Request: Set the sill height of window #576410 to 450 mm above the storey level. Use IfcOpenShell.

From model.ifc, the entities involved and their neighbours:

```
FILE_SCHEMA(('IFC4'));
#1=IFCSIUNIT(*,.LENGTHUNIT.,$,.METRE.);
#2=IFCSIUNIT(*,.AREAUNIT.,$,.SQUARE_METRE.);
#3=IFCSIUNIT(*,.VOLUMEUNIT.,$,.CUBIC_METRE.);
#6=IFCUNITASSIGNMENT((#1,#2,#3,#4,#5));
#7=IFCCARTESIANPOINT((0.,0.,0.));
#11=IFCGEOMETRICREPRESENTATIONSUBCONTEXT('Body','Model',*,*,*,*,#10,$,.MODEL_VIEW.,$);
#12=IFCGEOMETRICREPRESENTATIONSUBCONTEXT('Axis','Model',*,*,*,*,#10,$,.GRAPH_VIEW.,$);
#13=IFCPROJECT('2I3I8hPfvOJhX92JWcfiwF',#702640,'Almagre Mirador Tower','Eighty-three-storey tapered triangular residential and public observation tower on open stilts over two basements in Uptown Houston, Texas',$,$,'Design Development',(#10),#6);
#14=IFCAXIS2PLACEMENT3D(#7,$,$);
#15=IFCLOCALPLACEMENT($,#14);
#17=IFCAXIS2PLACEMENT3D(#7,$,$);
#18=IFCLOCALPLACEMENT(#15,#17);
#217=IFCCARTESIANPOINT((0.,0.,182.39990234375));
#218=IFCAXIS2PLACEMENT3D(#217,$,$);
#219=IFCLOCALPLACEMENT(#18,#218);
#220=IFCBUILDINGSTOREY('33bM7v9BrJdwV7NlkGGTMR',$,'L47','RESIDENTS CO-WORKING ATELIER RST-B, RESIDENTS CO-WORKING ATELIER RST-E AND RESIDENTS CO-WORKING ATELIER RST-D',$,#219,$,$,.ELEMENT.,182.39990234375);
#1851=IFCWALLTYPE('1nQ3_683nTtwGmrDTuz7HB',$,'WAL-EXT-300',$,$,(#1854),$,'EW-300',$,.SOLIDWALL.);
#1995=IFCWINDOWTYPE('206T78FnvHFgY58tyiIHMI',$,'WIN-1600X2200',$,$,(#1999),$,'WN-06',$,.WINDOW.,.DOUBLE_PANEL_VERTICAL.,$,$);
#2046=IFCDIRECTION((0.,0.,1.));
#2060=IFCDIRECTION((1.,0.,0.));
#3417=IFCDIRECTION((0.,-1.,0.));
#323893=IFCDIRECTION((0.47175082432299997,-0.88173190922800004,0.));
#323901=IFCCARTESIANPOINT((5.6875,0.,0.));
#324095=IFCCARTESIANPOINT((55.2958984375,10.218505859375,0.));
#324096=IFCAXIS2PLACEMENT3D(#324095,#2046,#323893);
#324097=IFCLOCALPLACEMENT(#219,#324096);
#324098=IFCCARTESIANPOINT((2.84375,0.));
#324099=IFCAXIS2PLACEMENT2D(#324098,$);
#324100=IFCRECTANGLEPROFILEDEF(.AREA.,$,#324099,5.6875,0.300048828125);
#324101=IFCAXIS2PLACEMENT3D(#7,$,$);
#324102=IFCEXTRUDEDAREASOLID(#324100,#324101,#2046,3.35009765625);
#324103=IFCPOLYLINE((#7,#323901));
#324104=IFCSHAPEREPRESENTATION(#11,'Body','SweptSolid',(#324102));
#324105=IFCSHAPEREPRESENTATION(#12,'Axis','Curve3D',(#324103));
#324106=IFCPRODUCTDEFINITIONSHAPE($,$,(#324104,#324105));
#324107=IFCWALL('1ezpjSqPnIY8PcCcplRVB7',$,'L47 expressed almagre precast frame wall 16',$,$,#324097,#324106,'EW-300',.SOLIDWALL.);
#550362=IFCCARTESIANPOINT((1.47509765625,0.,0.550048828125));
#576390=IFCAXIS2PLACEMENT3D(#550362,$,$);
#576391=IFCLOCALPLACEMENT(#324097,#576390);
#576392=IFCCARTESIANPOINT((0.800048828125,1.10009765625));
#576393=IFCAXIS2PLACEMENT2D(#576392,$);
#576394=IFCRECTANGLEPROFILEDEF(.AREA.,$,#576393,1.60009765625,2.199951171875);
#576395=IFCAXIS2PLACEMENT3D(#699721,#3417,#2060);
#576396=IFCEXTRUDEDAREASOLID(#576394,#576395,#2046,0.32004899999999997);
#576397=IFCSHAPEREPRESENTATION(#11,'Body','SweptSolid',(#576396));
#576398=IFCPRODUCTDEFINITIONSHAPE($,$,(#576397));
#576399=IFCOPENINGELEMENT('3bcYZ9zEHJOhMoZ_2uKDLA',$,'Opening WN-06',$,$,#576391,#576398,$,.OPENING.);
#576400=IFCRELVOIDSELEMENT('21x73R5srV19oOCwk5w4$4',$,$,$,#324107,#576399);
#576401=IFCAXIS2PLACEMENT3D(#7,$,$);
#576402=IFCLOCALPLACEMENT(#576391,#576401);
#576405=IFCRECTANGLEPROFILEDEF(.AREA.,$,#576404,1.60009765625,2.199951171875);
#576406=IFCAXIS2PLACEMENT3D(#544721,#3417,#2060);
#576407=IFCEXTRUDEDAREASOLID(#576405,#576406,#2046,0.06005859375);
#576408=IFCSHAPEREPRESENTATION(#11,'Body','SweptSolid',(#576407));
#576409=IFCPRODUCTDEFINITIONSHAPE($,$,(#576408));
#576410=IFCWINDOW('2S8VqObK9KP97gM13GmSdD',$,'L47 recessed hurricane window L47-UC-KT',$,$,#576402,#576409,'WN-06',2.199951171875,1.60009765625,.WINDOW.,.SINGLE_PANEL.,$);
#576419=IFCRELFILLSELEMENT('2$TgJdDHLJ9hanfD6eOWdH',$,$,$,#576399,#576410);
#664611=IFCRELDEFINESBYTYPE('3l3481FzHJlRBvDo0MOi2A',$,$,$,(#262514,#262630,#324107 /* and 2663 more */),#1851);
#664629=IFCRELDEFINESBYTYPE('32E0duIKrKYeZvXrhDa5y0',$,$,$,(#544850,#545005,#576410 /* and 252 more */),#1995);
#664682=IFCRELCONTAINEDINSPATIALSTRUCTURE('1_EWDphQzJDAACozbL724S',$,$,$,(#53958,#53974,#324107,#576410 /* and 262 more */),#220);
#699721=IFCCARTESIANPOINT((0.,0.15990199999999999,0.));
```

```python
import numpy as np
import ifcopenshell
import ifcopenshell.api.geometry
import ifcopenshell.geom
import ifcopenshell.util.element
import ifcopenshell.util.placement
import ifcopenshell.util.shape
import ifcopenshell.util.unit

model = ifcopenshell.open("model.ifc")
unit_scale = ifcopenshell.util.unit.calculate_unit_scale(model)

window = model.by_guid("2S8VqObK9KP97gM13GmSdD")
opening = window.FillsVoids[0].RelatingOpeningElement
storey = ifcopenshell.util.element.get_container(window, ifc_class="IfcBuildingStorey")
level = ifcopenshell.util.placement.get_local_placement(storey.ObjectPlacement)[2, 3]

# The opening's origin need not be at the sill, so measure its lowest point.
shape = ifcopenshell.geom.create_shape(ifcopenshell.geom.settings(), opening)
bottom = ifcopenshell.util.shape.get_shape_bottom_elevation(shape, shape.geometry) / unit_scale
dz = level + 0.45 - bottom

shift = np.array([0.0, 0.0, dz])
# The window is placed relative to its opening, so it follows when the opening moves.
matrix = ifcopenshell.util.placement.get_local_placement(opening.ObjectPlacement)
matrix[:3, 3] += shift
ifcopenshell.api.geometry.edit_object_placement(
    model, product=opening, matrix=matrix, is_si=False, should_transform_children=True
)

print(f"moved by {dz * unit_scale:+.3f} m")

model.write("model_edited.ifc")
```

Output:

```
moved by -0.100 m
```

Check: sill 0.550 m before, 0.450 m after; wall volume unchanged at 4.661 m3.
